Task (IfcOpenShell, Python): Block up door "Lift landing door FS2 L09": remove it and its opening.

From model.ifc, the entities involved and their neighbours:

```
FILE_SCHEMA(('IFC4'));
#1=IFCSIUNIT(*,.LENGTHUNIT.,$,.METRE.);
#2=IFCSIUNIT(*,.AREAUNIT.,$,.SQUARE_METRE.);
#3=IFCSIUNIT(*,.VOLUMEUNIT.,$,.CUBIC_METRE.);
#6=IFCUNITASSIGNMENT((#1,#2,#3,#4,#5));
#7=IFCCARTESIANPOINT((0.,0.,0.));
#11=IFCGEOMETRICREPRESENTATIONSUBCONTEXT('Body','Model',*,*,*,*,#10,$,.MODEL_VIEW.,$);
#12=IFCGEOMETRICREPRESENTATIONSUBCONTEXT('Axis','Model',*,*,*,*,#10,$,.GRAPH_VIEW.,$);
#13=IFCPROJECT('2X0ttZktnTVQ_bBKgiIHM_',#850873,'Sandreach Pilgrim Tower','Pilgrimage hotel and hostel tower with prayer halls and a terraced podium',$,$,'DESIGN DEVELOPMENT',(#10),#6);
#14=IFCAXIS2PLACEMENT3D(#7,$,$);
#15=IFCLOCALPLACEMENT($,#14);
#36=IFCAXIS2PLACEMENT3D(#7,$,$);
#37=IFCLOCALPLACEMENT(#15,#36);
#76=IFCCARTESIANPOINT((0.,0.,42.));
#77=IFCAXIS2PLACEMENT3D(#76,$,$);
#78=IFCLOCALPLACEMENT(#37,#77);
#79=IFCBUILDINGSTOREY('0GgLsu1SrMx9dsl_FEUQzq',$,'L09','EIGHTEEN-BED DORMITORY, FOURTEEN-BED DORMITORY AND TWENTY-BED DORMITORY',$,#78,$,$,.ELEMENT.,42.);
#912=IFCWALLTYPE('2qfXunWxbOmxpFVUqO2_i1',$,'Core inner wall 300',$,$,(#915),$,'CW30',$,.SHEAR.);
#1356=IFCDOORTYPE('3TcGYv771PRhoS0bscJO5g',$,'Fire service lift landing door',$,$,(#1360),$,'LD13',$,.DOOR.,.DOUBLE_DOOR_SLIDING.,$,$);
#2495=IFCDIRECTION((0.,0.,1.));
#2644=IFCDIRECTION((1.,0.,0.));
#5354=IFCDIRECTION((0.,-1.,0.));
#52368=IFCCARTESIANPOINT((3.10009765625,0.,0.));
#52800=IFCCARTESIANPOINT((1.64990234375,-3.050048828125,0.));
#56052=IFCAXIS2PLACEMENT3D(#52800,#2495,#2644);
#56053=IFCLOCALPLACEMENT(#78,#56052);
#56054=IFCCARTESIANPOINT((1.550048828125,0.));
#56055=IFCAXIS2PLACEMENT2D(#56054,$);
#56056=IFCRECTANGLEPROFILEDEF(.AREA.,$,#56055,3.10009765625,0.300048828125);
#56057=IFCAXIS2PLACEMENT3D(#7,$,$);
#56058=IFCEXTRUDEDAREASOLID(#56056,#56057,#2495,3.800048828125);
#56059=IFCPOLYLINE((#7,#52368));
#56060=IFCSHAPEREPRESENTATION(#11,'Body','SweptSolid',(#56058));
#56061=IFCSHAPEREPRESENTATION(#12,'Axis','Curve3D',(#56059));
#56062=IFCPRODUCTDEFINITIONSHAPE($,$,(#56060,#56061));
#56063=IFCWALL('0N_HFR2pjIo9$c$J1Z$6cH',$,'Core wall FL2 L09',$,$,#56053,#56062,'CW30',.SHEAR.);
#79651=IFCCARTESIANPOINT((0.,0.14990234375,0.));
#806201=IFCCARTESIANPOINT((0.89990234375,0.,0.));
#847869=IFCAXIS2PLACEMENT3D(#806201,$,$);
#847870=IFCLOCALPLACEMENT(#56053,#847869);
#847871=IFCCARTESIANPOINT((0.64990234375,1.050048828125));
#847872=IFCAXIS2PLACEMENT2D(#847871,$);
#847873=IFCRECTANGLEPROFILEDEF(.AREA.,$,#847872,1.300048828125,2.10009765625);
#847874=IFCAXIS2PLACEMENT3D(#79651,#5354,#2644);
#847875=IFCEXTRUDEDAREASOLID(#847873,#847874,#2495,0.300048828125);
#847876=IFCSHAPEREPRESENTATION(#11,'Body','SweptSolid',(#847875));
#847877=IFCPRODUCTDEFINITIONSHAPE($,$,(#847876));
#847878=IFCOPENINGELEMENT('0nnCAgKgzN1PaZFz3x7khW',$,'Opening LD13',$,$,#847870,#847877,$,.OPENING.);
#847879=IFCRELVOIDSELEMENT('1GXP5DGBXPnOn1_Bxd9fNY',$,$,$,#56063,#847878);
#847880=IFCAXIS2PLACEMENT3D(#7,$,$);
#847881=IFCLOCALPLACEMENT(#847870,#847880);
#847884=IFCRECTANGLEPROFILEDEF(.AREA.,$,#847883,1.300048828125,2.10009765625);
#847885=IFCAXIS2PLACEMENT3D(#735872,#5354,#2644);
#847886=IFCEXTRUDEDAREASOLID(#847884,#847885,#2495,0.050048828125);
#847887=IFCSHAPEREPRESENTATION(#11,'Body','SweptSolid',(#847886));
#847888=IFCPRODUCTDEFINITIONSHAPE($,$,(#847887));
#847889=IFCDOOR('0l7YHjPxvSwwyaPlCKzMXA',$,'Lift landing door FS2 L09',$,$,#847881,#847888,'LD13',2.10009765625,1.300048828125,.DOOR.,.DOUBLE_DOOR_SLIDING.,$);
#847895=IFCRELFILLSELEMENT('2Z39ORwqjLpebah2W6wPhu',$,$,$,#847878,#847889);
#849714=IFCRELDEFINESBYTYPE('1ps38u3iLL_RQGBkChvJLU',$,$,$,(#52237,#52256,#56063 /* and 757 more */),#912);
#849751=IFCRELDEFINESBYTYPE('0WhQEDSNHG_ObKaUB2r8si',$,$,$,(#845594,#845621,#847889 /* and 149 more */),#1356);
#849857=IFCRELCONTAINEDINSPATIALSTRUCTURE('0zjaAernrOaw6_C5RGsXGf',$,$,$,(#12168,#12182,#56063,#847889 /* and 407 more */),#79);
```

```python
import ifcopenshell
import ifcopenshell.api.feature
import ifcopenshell.api.root
import ifcopenshell.geom
import ifcopenshell.util.shape

model = ifcopenshell.open("model.ifc")
settings = ifcopenshell.geom.settings()


def volume(element):
    """Net volume in cubic metres, openings subtracted."""
    shape = ifcopenshell.geom.create_shape(settings, element)
    return ifcopenshell.util.shape.get_volume(shape.geometry)


door = model.by_guid("0l7YHjPxvSwwyaPlCKzMXA")
opening = door.FillsVoids[0].RelatingOpeningElement
wall = opening.VoidsElements[0].RelatingBuildingElement
before = volume(wall)

ifcopenshell.api.root.remove_product(model, product=door)
ifcopenshell.api.feature.remove_feature(model, feature=opening)

after = volume(wall)

print(f"wall volume {before:.3f} -> {after:.3f} m3")

model.write("model_edited.ifc")
```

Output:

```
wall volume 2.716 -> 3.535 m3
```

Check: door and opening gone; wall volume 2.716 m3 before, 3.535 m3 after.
